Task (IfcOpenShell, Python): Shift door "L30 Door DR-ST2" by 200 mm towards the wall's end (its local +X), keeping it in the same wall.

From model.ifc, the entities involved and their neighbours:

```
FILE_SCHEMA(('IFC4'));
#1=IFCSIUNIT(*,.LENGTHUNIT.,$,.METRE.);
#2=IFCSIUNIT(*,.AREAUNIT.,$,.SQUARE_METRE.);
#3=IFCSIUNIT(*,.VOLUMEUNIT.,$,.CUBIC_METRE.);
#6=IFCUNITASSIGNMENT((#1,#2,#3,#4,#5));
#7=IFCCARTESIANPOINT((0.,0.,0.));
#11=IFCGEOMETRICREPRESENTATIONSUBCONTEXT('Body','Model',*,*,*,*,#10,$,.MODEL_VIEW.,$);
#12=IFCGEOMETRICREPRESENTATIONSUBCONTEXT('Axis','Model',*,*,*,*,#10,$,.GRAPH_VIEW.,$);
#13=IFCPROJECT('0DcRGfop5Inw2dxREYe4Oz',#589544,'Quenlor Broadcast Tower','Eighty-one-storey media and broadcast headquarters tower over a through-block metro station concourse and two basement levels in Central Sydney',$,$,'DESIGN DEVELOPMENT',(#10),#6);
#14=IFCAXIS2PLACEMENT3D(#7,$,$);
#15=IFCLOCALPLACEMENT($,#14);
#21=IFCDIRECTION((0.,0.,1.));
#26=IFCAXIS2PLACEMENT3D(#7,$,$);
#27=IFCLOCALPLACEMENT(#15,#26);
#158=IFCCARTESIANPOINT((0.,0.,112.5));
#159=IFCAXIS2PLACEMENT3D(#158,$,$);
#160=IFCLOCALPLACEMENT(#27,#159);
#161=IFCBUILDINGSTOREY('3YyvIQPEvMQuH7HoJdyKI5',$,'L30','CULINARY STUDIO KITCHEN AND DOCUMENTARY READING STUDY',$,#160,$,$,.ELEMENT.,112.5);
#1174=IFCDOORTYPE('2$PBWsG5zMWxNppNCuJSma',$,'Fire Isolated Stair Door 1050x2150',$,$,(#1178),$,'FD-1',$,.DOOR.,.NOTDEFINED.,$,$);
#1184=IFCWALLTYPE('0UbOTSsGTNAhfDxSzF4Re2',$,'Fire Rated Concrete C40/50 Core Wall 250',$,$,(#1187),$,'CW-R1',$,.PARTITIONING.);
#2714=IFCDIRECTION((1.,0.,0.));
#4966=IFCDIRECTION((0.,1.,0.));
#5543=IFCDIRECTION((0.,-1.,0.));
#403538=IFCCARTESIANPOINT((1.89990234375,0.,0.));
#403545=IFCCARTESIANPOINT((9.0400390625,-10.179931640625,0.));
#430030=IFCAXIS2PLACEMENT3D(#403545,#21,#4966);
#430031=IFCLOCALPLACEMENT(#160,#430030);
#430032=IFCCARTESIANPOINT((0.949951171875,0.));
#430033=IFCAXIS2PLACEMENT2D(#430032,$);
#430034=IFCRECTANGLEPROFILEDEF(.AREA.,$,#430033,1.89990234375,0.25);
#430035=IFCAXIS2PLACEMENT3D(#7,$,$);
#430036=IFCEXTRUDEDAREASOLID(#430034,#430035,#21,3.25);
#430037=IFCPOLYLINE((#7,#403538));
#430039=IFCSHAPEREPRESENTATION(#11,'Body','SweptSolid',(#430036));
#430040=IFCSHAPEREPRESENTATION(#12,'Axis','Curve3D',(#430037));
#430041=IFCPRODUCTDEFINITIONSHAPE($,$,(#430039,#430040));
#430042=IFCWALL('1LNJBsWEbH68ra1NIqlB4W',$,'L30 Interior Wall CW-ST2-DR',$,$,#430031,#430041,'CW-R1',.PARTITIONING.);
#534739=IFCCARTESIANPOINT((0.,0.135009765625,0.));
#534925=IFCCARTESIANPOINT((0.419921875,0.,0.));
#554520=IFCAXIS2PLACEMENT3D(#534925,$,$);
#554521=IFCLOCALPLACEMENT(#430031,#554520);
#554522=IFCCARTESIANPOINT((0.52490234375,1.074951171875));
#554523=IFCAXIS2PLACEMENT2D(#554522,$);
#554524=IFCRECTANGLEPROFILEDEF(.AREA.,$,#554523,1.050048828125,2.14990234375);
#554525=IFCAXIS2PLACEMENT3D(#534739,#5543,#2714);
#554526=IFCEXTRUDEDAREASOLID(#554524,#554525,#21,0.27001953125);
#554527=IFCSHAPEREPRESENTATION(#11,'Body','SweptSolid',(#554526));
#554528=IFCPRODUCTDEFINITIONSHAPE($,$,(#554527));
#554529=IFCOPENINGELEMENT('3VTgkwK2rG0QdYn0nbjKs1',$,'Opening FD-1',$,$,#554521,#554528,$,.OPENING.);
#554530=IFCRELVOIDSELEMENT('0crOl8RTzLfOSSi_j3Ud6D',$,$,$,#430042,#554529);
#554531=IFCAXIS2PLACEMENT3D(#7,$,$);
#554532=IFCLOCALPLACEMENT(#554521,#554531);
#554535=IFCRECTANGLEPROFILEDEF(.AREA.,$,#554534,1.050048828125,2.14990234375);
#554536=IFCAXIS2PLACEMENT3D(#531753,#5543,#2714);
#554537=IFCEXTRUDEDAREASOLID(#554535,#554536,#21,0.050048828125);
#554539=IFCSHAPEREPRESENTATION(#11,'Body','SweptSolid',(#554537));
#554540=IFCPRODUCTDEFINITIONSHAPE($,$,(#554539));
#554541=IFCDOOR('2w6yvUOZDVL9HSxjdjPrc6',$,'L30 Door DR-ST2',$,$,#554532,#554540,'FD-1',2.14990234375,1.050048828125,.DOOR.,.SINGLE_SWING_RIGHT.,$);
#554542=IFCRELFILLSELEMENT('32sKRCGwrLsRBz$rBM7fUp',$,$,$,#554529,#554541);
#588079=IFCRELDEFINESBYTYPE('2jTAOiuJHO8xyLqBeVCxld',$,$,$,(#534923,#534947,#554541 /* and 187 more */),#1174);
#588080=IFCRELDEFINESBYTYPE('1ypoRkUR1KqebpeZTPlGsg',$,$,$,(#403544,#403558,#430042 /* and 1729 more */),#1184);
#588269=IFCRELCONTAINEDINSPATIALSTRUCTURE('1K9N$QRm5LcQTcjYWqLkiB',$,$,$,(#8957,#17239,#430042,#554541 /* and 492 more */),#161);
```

```python
import ifcopenshell
import ifcopenshell.api.geometry
import ifcopenshell.util.placement
import ifcopenshell.util.unit

model = ifcopenshell.open("model.ifc")
unit_scale = ifcopenshell.util.unit.calculate_unit_scale(model)

door = model.by_guid("2w6yvUOZDVL9HSxjdjPrc6")
opening = door.FillsVoids[0].RelatingOpeningElement
wall = opening.VoidsElements[0].RelatingBuildingElement

wall_matrix = ifcopenshell.util.placement.get_local_placement(wall.ObjectPlacement)
shift = wall_matrix[:3, 0] * 0.2 / unit_scale
before = ifcopenshell.util.placement.get_local_placement(door.ObjectPlacement)[:3, 3].copy()

# The door is placed relative to its opening, so it follows when the opening moves.
matrix = ifcopenshell.util.placement.get_local_placement(opening.ObjectPlacement)
matrix[:3, 3] += shift
ifcopenshell.api.geometry.edit_object_placement(
    model, product=opening, matrix=matrix, is_si=False, should_transform_children=True
)

after = ifcopenshell.util.placement.get_local_placement(door.ObjectPlacement)[:3, 3]
print("door moved by", (after - before).round(3) + 0.0)

model.write("model_rev.ifc")
```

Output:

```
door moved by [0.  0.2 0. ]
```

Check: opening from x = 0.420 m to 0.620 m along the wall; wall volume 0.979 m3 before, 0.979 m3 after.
